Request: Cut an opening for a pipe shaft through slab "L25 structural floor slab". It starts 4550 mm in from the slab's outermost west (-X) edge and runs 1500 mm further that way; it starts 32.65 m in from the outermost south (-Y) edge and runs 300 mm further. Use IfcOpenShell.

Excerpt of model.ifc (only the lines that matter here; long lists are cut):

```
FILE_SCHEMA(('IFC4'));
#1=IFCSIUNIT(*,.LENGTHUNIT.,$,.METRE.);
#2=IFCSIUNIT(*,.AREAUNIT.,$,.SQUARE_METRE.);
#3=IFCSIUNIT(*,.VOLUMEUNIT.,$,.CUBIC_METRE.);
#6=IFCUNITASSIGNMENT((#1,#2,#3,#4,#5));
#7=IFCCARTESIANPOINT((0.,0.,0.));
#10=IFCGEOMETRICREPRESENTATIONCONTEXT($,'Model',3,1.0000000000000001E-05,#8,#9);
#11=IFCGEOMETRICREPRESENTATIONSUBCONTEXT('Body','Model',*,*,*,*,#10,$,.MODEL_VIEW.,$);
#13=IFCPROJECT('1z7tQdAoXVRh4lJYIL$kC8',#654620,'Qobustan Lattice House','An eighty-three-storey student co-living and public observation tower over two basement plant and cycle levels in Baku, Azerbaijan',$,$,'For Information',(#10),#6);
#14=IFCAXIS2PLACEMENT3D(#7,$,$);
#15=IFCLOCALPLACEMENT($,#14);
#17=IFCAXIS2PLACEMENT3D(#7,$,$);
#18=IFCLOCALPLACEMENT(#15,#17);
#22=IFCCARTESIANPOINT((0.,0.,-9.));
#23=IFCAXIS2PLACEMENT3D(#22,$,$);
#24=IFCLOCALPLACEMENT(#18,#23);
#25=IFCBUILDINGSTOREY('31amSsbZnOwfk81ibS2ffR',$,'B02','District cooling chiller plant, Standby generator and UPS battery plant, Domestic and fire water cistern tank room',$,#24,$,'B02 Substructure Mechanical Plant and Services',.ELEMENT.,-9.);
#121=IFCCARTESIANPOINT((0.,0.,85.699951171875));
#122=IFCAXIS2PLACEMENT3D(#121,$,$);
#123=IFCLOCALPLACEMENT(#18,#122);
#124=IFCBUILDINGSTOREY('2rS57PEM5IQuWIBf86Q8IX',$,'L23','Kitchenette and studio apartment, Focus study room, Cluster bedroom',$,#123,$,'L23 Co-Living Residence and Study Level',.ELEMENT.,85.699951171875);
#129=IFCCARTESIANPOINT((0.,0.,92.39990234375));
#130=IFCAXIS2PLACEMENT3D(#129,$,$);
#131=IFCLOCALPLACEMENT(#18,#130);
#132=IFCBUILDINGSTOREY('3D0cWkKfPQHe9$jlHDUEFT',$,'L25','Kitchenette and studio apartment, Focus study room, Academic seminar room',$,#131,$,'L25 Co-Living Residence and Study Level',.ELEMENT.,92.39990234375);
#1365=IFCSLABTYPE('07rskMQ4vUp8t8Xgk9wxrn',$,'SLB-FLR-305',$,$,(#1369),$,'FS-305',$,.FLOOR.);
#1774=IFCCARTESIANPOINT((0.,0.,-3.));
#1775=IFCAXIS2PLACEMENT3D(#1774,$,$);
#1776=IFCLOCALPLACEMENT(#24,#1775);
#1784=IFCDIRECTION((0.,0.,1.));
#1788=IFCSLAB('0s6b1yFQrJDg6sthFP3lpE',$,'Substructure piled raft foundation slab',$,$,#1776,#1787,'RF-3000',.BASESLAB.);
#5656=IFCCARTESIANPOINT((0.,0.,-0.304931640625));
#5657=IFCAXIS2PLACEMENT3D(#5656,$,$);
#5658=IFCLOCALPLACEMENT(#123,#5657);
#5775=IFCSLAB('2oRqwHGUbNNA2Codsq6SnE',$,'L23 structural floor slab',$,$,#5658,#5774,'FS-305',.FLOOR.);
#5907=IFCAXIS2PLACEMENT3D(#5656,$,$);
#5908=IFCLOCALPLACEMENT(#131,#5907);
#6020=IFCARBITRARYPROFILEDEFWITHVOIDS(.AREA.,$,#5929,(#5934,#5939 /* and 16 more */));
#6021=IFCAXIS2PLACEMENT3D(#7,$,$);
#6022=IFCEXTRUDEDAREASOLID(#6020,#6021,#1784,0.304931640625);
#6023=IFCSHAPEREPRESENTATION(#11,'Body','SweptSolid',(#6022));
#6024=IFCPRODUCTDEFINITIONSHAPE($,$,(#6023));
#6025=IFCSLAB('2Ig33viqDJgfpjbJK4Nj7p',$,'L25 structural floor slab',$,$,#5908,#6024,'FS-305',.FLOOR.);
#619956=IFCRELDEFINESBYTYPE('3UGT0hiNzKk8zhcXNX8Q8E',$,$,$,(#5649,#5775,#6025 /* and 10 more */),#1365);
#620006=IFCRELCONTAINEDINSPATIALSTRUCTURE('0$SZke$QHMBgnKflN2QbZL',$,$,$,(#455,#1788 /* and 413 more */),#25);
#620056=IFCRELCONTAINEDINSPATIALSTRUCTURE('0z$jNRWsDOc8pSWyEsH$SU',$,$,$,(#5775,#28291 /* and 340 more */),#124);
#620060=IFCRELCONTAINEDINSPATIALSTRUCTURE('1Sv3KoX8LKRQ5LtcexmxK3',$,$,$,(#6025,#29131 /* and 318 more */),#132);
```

```python
import numpy as np
import ifcopenshell
import ifcopenshell.api.feature
import ifcopenshell.api.geometry
import ifcopenshell.api.root
import ifcopenshell.geom
import ifcopenshell.util.placement
import ifcopenshell.util.representation
import ifcopenshell.util.shape
import ifcopenshell.util.unit

model = ifcopenshell.open("model.ifc")
unit_scale = ifcopenshell.util.unit.calculate_unit_scale(model)
settings = ifcopenshell.geom.settings()


def volume(element):
    """Net volume in cubic metres, openings subtracted."""
    shape = ifcopenshell.geom.create_shape(settings, element)
    return ifcopenshell.util.shape.get_volume(shape.geometry)


slab = model.by_id(6025)
before = volume(slab)

# Extent in the slab's own axes, in metres. The edges named are its -X and -Y sides.
slab_shape = ifcopenshell.geom.create_shape(settings, slab)
vertices = ifcopenshell.util.shape.get_vertices(slab_shape.geometry)
x_min, y_min, bottom = vertices.min(axis=0)
top = vertices[:, 2].max()

opening = ifcopenshell.api.root.create_entity(model, ifc_class="IfcOpeningElement", name="Pipe shaft opening", predefined_type="OPENING")
context = ifcopenshell.util.representation.get_context(model, "Model", "Body", "MODEL_VIEW")
width, depth = 1.5, 0.3
outline = [(0.0, 0.0), (width, 0.0), (width, depth), (0.0, depth), (0.0, 0.0)]
# Overshoot both faces by 50 mm so the cut is clean.
shape = ifcopenshell.api.geometry.add_slab_representation(
    model, context=context, depth=top - bottom + 0.1, polyline=outline
)
ifcopenshell.api.geometry.assign_representation(model, product=opening, representation=shape)

matrix = ifcopenshell.util.placement.get_local_placement(slab.ObjectPlacement)
matrix[:, 3] = matrix @ np.append(np.array([x_min + 4.55, y_min + 32.65, bottom - 0.05]) / unit_scale, 1.0)
ifcopenshell.api.geometry.edit_object_placement(model, product=opening, matrix=matrix, is_si=False)
ifcopenshell.api.feature.add_feature(model, feature=opening, element=slab)

after = volume(slab)

print(f"slab volume {before:.3f} -> {after:.3f} m3")

model.write("model_rev.ifc")
```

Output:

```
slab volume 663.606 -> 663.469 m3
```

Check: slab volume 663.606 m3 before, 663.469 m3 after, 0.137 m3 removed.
